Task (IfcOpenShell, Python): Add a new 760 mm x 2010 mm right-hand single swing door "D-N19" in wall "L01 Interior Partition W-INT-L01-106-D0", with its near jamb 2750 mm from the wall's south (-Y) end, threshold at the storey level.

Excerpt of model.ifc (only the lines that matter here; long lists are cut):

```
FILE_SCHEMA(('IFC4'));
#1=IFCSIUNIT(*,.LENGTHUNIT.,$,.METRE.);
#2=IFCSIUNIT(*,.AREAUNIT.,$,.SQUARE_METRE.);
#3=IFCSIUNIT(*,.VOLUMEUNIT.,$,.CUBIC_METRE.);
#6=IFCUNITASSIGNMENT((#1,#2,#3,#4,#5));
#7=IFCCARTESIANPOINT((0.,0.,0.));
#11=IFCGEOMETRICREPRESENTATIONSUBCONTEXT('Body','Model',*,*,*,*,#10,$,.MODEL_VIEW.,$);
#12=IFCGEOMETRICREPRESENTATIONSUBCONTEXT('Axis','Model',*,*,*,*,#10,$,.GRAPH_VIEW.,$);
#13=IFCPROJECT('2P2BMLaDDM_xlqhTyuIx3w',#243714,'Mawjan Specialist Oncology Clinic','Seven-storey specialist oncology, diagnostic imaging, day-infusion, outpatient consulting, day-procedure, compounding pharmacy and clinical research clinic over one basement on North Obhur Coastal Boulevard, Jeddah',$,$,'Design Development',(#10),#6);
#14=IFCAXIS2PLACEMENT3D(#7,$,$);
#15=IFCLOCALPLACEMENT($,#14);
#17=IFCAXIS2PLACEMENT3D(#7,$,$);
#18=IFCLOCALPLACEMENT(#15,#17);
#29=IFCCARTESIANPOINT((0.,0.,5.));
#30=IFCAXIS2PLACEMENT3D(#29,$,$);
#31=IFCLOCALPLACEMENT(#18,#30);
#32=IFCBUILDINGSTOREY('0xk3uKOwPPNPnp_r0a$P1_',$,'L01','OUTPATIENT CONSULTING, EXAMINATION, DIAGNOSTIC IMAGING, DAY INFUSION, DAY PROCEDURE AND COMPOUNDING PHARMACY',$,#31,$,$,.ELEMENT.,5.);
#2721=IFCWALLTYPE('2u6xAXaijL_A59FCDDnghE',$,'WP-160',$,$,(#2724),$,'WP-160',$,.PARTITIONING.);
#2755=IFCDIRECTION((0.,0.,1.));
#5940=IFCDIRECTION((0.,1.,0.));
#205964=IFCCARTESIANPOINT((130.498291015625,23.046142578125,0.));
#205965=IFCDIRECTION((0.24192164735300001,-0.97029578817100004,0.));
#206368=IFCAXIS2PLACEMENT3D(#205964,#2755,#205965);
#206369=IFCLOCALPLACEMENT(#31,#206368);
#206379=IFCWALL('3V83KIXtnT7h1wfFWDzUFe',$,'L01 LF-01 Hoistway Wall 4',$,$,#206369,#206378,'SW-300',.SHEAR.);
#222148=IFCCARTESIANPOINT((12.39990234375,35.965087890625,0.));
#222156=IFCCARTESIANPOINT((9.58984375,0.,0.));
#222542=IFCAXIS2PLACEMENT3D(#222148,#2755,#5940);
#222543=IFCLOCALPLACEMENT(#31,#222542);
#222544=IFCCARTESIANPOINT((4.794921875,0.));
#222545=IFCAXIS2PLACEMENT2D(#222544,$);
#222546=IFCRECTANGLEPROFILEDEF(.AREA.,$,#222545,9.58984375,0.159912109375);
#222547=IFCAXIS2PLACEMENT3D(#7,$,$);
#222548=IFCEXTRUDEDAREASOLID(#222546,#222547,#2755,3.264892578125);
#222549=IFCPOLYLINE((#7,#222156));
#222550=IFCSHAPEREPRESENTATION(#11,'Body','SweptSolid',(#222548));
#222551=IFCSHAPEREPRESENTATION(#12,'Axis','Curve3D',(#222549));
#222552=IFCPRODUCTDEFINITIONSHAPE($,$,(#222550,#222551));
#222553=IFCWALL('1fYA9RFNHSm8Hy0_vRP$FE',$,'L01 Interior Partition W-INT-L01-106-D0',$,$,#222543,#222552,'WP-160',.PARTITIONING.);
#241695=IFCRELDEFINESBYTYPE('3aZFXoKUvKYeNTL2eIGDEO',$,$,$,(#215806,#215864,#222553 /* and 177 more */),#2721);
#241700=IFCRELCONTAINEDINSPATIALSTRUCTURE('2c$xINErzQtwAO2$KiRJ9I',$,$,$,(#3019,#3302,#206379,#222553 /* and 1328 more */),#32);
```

```python
import numpy as np
import ifcopenshell
import ifcopenshell.api.feature
import ifcopenshell.api.geometry
import ifcopenshell.api.root
import ifcopenshell.api.spatial
import ifcopenshell.geom
import ifcopenshell.util.element
import ifcopenshell.util.placement
import ifcopenshell.util.representation
import ifcopenshell.util.shape
import ifcopenshell.util.unit

model = ifcopenshell.open("model.ifc")
unit_scale = ifcopenshell.util.unit.calculate_unit_scale(model)
settings = ifcopenshell.geom.settings()


def volume(element):
    """Net volume in cubic metres, openings subtracted."""
    shape = ifcopenshell.geom.create_shape(settings, element)
    return ifcopenshell.util.shape.get_volume(shape.geometry)


wall = model.by_guid("1fYA9RFNHSm8Hy0_vRP$FE")
storey = ifcopenshell.util.element.get_container(wall, ifc_class="IfcBuildingStorey")
context = ifcopenshell.util.representation.get_context(model, "Model", "Body", "MODEL_VIEW")
before = volume(wall)

width, height, from_end, sill = 0.76, 2.01, 2.75, 0.0  # metres

# The wall runs along its own X axis, and the end named is its -X end.
wall_shape = ifcopenshell.geom.create_shape(settings, wall)
x, y, z = ifcopenshell.util.shape.get_vertices(wall_shape.geometry).T
start = x.min() + from_end
face, thickness = float(y.min()), float(y.max() - y.min())
wall_matrix = ifcopenshell.util.placement.get_local_placement(wall.ObjectPlacement)
level = ifcopenshell.util.placement.get_local_placement(storey.ObjectPlacement)[2, 3]


def in_wall(x, y):
    """Placement at x, y metres in the wall's axes, at sill height."""
    matrix = wall_matrix.copy()
    matrix[:, 3] = wall_matrix @ np.array([x / unit_scale, y / unit_scale, 0.0, 1.0])
    matrix[2, 3] = level + sill / unit_scale
    return matrix


# Opening: a box that overshoots both wall faces by 50 mm.
opening = ifcopenshell.api.root.create_entity(model, ifc_class="IfcOpeningElement", predefined_type="OPENING")
box = ifcopenshell.api.geometry.add_wall_representation(
    model, context=context, length=width, height=height, thickness=thickness + 0.1
)
ifcopenshell.api.geometry.assign_representation(model, product=opening, representation=box)
ifcopenshell.api.geometry.edit_object_placement(model, product=opening, matrix=in_wall(start, face - 0.05), is_si=False)
ifcopenshell.api.feature.add_feature(model, feature=opening, element=wall)

door = ifcopenshell.api.root.create_entity(model, ifc_class="IfcDoor", name="D-N19", predefined_type="DOOR")
door.OverallWidth, door.OverallHeight = width / unit_scale, height / unit_scale
door.OperationType = "SINGLE_SWING_RIGHT"
body = ifcopenshell.api.geometry.add_door_representation(
    model,
    context=context,
    overall_width=door.OverallWidth,
    overall_height=door.OverallHeight,
    operation_type="SINGLE_SWING_RIGHT",
    lining_properties={"LiningDepth": thickness / unit_scale, "ThresholdDepth": thickness / unit_scale},
)
ifcopenshell.api.geometry.assign_representation(model, product=door, representation=body)
ifcopenshell.api.spatial.assign_container(model, products=[door], relating_structure=storey)
ifcopenshell.api.feature.add_filling(model, opening=opening, element=door)

# The lining spans the wall, so the door starts at the wall face.
ifcopenshell.api.geometry.edit_object_placement(model, product=door, matrix=in_wall(start, face), is_si=False)

after = volume(wall)

print(f"wall volume {before:.3f} -> {after:.3f} m3")

model.write("model_v2.ifc")
```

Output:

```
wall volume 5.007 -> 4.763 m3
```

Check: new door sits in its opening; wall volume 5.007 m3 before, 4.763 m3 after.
